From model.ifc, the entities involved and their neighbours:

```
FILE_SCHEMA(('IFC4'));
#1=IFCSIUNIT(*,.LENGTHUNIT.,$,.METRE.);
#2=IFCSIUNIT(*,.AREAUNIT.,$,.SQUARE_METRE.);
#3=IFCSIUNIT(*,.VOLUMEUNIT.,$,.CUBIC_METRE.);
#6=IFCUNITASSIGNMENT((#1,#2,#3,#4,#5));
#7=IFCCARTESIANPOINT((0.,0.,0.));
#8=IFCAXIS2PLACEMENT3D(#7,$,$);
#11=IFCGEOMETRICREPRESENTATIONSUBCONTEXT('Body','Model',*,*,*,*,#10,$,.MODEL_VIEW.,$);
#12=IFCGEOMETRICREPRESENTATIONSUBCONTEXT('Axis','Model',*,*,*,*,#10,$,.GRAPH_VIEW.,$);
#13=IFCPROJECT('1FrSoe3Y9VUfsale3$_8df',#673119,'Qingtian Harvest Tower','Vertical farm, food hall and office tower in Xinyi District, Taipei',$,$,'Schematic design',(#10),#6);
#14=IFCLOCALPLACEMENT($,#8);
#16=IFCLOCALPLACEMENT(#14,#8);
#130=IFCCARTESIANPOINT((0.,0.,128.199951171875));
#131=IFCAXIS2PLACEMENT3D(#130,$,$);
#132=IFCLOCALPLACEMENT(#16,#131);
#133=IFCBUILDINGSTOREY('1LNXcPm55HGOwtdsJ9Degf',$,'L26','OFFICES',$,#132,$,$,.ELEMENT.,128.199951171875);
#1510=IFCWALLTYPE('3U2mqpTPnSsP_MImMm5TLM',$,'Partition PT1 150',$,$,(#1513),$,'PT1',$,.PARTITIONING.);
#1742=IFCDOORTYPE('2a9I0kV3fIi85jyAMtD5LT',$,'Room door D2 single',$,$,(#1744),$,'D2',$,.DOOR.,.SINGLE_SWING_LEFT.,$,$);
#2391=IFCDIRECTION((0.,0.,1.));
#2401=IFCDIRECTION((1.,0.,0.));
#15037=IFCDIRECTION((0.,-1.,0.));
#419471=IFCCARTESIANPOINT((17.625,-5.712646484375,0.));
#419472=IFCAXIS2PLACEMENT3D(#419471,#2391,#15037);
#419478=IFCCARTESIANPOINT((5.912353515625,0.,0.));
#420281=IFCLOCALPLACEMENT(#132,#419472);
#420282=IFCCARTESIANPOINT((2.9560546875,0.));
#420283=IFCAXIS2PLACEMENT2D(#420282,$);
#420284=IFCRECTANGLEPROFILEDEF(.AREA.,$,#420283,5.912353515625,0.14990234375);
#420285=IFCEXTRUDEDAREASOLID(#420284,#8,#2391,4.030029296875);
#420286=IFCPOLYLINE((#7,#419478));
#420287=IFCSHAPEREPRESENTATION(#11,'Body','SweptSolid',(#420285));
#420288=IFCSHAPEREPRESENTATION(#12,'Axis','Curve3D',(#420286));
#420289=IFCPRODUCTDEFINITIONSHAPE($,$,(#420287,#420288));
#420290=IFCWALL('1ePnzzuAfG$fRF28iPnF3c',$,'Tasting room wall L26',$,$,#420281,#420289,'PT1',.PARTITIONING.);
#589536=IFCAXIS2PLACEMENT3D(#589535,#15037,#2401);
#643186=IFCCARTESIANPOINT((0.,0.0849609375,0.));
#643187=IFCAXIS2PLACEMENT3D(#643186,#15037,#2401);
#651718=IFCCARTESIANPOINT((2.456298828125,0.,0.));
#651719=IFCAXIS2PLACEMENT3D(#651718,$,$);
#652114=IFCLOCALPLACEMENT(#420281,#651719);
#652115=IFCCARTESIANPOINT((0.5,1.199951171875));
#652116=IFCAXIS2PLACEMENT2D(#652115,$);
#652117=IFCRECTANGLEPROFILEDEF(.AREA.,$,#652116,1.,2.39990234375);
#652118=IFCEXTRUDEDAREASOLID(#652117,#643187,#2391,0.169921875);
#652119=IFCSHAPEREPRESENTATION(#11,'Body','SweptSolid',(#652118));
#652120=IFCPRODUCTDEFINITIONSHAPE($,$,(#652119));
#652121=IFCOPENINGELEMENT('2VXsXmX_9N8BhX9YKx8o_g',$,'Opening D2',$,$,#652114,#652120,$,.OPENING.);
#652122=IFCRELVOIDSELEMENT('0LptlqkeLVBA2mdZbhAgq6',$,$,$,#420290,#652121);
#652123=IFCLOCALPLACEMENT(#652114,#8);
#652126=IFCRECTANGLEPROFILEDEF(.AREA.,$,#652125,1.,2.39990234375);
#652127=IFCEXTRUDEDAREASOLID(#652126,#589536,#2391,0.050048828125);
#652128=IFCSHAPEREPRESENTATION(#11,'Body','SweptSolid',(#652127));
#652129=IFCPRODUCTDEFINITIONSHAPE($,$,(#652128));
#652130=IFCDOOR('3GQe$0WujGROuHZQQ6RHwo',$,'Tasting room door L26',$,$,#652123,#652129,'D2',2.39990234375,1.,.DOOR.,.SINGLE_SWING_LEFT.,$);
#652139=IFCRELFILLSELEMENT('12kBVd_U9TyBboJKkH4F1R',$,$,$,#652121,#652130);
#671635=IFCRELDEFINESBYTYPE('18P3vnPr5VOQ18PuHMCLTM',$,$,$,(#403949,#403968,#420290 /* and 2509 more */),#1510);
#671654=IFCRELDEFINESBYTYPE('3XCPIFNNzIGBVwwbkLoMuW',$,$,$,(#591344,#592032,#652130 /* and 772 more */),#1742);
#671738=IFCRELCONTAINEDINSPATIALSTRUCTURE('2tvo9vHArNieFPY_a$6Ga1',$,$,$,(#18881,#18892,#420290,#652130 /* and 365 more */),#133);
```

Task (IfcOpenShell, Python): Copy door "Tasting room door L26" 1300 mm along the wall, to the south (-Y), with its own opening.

```python
import ifcopenshell
import ifcopenshell.api.feature
import ifcopenshell.api.geometry
import ifcopenshell.api.root
import ifcopenshell.geom
import ifcopenshell.util.element
import ifcopenshell.util.placement
import ifcopenshell.util.shape

model = ifcopenshell.open("model.ifc")
settings = ifcopenshell.geom.settings()


def volume(element):
    """Net volume in cubic metres, openings subtracted."""
    shape = ifcopenshell.geom.create_shape(settings, element)
    return ifcopenshell.util.shape.get_volume(shape.geometry)


door = model.by_guid("3GQe$0WujGROuHZQQ6RHwo")
opening = door.FillsVoids[0].RelatingOpeningElement
wall = opening.VoidsElements[0].RelatingBuildingElement
before = volume(wall)
shift = ifcopenshell.util.placement.get_local_placement(wall.ObjectPlacement)[:3, 0] * 1.3

# copy_class copies the void relationship, type, container and properties, but no geometry.
new_opening = ifcopenshell.api.root.copy_class(model, product=opening)
new_opening.Representation = ifcopenshell.util.element.copy_deep(
    model, opening.Representation, exclude=["IfcGeometricRepresentationContext", "IfcRepresentationMap"]
)
new_door = ifcopenshell.api.root.copy_class(model, product=door)
new_door.Representation = ifcopenshell.util.element.copy_deep(
    model, door.Representation, exclude=["IfcGeometricRepresentationContext", "IfcRepresentationMap"]
)
new_door.Tag = None
ifcopenshell.api.feature.add_filling(model, opening=new_opening, element=new_door)

for old, new in ((opening, new_opening), (door, new_door)):
    matrix = ifcopenshell.util.placement.get_local_placement(old.ObjectPlacement)
    matrix[:3, 3] += shift
    ifcopenshell.api.geometry.edit_object_placement(model, product=new, matrix=matrix, is_si=False)

after = volume(wall)

print(f"wall volume {before:.3f} -> {after:.3f} m3")

model.write("model_v2.ifc")
```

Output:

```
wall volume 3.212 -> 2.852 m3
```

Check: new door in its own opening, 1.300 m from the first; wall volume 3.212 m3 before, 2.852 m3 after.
